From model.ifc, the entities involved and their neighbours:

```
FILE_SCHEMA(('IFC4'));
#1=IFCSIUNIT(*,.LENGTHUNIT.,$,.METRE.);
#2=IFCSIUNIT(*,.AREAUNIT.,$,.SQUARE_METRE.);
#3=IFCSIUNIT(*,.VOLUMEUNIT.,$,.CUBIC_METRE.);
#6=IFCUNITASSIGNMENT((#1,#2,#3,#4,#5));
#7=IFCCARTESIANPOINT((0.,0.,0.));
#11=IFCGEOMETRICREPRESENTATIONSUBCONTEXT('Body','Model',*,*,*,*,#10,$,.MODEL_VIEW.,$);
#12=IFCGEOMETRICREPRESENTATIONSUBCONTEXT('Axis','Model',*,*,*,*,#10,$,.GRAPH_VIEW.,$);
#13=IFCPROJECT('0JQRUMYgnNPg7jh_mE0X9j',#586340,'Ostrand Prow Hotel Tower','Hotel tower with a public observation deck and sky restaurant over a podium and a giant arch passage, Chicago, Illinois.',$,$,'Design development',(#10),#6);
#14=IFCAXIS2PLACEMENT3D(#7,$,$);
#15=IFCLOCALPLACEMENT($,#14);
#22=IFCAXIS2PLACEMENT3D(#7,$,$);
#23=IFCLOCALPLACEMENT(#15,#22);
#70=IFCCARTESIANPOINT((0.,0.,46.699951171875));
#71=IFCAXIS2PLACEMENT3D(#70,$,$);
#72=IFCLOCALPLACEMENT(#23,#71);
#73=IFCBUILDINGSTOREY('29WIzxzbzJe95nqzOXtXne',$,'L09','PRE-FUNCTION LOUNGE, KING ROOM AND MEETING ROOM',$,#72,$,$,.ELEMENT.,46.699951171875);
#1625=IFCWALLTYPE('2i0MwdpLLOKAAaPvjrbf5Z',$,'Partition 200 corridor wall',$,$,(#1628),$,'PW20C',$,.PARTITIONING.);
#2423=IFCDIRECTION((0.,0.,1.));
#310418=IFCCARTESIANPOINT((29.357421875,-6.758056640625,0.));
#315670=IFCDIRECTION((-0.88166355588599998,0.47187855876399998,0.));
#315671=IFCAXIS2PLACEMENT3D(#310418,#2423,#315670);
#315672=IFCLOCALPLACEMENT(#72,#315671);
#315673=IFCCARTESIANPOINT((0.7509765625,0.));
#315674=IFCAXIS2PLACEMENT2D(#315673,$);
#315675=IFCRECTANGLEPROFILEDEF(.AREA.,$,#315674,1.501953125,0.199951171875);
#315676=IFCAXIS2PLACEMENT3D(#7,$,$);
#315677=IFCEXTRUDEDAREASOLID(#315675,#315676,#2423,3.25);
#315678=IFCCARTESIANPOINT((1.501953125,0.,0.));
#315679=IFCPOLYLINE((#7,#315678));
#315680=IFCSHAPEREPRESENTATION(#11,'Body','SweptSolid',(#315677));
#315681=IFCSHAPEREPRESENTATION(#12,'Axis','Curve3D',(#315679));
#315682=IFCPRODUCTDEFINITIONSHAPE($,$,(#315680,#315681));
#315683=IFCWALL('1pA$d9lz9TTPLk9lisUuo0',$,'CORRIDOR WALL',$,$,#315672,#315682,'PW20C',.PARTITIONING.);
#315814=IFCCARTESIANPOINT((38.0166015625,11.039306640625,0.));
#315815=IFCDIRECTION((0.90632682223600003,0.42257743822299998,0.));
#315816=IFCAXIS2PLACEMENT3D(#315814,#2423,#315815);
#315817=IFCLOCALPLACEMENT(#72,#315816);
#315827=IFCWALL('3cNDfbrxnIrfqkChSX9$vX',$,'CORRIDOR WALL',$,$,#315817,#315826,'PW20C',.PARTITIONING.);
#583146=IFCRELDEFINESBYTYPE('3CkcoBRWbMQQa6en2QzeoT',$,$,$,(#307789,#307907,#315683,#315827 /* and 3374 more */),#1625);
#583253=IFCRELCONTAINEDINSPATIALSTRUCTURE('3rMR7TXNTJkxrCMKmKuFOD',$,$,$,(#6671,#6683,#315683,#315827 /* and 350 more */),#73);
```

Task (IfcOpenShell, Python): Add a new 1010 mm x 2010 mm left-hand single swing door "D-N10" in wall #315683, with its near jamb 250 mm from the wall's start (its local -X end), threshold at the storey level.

```python
import numpy as np
import ifcopenshell
import ifcopenshell.api.feature
import ifcopenshell.api.geometry
import ifcopenshell.api.root
import ifcopenshell.api.spatial
import ifcopenshell.geom
import ifcopenshell.util.element
import ifcopenshell.util.placement
import ifcopenshell.util.representation
import ifcopenshell.util.shape
import ifcopenshell.util.unit

model = ifcopenshell.open("model.ifc")
unit_scale = ifcopenshell.util.unit.calculate_unit_scale(model)
settings = ifcopenshell.geom.settings()


def volume(element):
    """Net volume in cubic metres, openings subtracted."""
    shape = ifcopenshell.geom.create_shape(settings, element)
    return ifcopenshell.util.shape.get_volume(shape.geometry)


wall = model.by_id(315683)
storey = ifcopenshell.util.element.get_container(wall, ifc_class="IfcBuildingStorey")
context = ifcopenshell.util.representation.get_context(model, "Model", "Body", "MODEL_VIEW")
before = volume(wall)

width, height, from_end, sill = 1.01, 2.01, 0.25, 0.0  # metres

# The wall runs along its own X axis, and the end named is its -X end.
wall_shape = ifcopenshell.geom.create_shape(settings, wall)
x, y, z = ifcopenshell.util.shape.get_vertices(wall_shape.geometry).T
start = x.min() + from_end
face, thickness = float(y.min()), float(y.max() - y.min())
wall_matrix = ifcopenshell.util.placement.get_local_placement(wall.ObjectPlacement)
level = ifcopenshell.util.placement.get_local_placement(storey.ObjectPlacement)[2, 3]


def in_wall(x, y):
    """Placement at x, y metres in the wall's axes, at sill height."""
    matrix = wall_matrix.copy()
    matrix[:, 3] = wall_matrix @ np.array([x / unit_scale, y / unit_scale, 0.0, 1.0])
    matrix[2, 3] = level + sill / unit_scale
    return matrix


# Opening: a box that overshoots both wall faces by 50 mm.
opening = ifcopenshell.api.root.create_entity(model, ifc_class="IfcOpeningElement", predefined_type="OPENING")
box = ifcopenshell.api.geometry.add_wall_representation(
    model, context=context, length=width, height=height, thickness=thickness + 0.1
)
ifcopenshell.api.geometry.assign_representation(model, product=opening, representation=box)
ifcopenshell.api.geometry.edit_object_placement(model, product=opening, matrix=in_wall(start, face - 0.05), is_si=False)
ifcopenshell.api.feature.add_feature(model, feature=opening, element=wall)

door = ifcopenshell.api.root.create_entity(model, ifc_class="IfcDoor", name="D-N10", predefined_type="DOOR")
door.OverallWidth, door.OverallHeight = width / unit_scale, height / unit_scale
door.OperationType = "SINGLE_SWING_LEFT"
body = ifcopenshell.api.geometry.add_door_representation(
    model,
    context=context,
    overall_width=door.OverallWidth,
    overall_height=door.OverallHeight,
    operation_type="SINGLE_SWING_LEFT",
    lining_properties={"LiningDepth": thickness / unit_scale, "ThresholdDepth": thickness / unit_scale},
)
ifcopenshell.api.geometry.assign_representation(model, product=door, representation=body)
ifcopenshell.api.spatial.assign_container(model, products=[door], relating_structure=storey)
ifcopenshell.api.feature.add_filling(model, opening=opening, element=door)

# The lining spans the wall, so the door starts at the wall face.
ifcopenshell.api.geometry.edit_object_placement(model, product=door, matrix=in_wall(start, face), is_si=False)

after = volume(wall)

print(f"wall volume {before:.3f} -> {after:.3f} m3")

model.write("model-out.ifc")
```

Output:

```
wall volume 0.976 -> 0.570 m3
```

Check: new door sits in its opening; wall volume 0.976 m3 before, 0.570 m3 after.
